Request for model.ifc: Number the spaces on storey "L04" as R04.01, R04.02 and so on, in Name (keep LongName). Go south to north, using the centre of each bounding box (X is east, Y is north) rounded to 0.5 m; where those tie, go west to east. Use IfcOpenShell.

First a look at what the model holds.

```python
import ifcopenshell
import ifcopenshell.util.element
import ifcopenshell.util.placement

model = ifcopenshell.open("model.ifc")
print(model.schema)
storey = next(s for s in model.by_type("IfcBuildingStorey") if s.Name == "L04")
spaces = [e for e in ifcopenshell.util.element.get_decomposition(storey) if e.is_a("IfcSpace")]
for e in sorted(spaces, key=lambda e: e.id()):
    origin = ifcopenshell.util.placement.get_local_placement(e.ObjectPlacement)[:3, 3]
    print(e.id(), e.Name, e.LongName, origin.round(2) + 0.0, sep=" | ")
```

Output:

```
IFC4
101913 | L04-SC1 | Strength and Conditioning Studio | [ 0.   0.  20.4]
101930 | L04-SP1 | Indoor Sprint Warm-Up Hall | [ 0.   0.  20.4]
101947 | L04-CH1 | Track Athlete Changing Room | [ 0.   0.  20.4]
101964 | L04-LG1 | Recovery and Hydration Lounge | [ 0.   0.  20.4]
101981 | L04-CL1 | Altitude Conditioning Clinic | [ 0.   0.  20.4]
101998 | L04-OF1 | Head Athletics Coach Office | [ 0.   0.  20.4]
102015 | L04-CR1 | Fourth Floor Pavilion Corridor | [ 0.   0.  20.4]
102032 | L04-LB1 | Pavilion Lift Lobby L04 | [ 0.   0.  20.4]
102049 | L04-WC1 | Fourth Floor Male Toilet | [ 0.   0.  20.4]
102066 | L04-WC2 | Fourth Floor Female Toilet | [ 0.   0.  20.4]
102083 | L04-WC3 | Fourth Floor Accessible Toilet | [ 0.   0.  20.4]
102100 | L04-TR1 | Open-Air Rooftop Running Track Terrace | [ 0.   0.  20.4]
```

```python
import ifcopenshell
import ifcopenshell.geom
import ifcopenshell.util.element
import ifcopenshell.util.shape

model = ifcopenshell.open("model.ifc")
settings = ifcopenshell.geom.settings()
settings.set("use-world-coords", True)


def centre(element):
    shape = ifcopenshell.geom.create_shape(settings, element)
    return ifcopenshell.util.shape.get_bbox_centroid(shape.geometry)


storey = next(s for s in model.by_type("IfcBuildingStorey") if s.Name == "L04")
spaces = [e for e in ifcopenshell.util.element.get_decomposition(storey) if e.is_a("IfcSpace")]

# Insertion points can sit at a corner or the storey origin, so sort by the geometry (in metres).
centres = {e: centre(e) for e in spaces}
spaces.sort(key=lambda e: (round(centres[e][1] / 0.5), centres[e][0]))

for i, e in enumerate(spaces, start=1):
    number = f"R04.{i:02d}"
    e.Name = number
    print(e.id(), number)

model.write("model_edited.ifc")
```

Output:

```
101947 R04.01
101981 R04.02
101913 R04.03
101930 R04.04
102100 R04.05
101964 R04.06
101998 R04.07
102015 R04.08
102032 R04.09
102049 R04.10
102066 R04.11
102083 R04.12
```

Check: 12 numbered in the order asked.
